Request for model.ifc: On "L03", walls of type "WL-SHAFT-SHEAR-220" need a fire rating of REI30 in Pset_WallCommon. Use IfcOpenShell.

First a look at what the model holds.

```python
import ifcopenshell
import ifcopenshell.util.element

model = ifcopenshell.open("model.ifc")
print(model.schema)
storey = next(s for s in model.by_type("IfcBuildingStorey") if s.Name == "L03")
walls = [e for e in ifcopenshell.util.element.get_decomposition(storey) if e.is_a("IfcWall")]
seen = {}
for e in walls:
    element_type = ifcopenshell.util.element.get_type(e)
    key = (element_type.Name if element_type != e and element_type else None, ifcopenshell.util.element.get_pset(e, "Pset_WallCommon", "FireRating"))
    seen[key] = seen.get(key, 0) + 1
for (name, value), count in sorted(seen.items(), key=str):
    print(count, "x", name, "|", value)
```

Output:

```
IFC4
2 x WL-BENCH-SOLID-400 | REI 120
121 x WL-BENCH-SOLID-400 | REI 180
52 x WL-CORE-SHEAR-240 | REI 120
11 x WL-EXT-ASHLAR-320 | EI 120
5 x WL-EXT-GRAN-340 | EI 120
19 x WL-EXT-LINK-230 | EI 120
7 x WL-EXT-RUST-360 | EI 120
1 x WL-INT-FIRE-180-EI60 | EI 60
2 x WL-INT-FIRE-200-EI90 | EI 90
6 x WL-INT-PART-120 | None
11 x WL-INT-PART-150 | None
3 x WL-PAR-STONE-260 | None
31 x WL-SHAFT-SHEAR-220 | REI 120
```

```python
import ifcopenshell
import ifcopenshell.api.pset
import ifcopenshell.util.element

model = ifcopenshell.open("model.ifc")

storey = next(s for s in model.by_type("IfcBuildingStorey") if s.Name == "L03")
walls = [e for e in ifcopenshell.util.element.get_decomposition(storey) if e.is_a("IfcWall")]

count = 0
for e in walls:
    element_type = ifcopenshell.util.element.get_type(e)
    if element_type in (None, e) or element_type.Name != "WL-SHAFT-SHEAR-220":
        continue
    # add_pset returns the element's existing set when there is one.
    pset = ifcopenshell.api.pset.add_pset(model, product=e, name="Pset_WallCommon")
    ifcopenshell.api.pset.edit_pset(model, pset=pset, properties={"FireRating": "REI30"})
    count += 1

print(count, "walls updated")

model.write("model_rev.ifc")
```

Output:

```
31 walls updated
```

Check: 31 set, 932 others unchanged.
